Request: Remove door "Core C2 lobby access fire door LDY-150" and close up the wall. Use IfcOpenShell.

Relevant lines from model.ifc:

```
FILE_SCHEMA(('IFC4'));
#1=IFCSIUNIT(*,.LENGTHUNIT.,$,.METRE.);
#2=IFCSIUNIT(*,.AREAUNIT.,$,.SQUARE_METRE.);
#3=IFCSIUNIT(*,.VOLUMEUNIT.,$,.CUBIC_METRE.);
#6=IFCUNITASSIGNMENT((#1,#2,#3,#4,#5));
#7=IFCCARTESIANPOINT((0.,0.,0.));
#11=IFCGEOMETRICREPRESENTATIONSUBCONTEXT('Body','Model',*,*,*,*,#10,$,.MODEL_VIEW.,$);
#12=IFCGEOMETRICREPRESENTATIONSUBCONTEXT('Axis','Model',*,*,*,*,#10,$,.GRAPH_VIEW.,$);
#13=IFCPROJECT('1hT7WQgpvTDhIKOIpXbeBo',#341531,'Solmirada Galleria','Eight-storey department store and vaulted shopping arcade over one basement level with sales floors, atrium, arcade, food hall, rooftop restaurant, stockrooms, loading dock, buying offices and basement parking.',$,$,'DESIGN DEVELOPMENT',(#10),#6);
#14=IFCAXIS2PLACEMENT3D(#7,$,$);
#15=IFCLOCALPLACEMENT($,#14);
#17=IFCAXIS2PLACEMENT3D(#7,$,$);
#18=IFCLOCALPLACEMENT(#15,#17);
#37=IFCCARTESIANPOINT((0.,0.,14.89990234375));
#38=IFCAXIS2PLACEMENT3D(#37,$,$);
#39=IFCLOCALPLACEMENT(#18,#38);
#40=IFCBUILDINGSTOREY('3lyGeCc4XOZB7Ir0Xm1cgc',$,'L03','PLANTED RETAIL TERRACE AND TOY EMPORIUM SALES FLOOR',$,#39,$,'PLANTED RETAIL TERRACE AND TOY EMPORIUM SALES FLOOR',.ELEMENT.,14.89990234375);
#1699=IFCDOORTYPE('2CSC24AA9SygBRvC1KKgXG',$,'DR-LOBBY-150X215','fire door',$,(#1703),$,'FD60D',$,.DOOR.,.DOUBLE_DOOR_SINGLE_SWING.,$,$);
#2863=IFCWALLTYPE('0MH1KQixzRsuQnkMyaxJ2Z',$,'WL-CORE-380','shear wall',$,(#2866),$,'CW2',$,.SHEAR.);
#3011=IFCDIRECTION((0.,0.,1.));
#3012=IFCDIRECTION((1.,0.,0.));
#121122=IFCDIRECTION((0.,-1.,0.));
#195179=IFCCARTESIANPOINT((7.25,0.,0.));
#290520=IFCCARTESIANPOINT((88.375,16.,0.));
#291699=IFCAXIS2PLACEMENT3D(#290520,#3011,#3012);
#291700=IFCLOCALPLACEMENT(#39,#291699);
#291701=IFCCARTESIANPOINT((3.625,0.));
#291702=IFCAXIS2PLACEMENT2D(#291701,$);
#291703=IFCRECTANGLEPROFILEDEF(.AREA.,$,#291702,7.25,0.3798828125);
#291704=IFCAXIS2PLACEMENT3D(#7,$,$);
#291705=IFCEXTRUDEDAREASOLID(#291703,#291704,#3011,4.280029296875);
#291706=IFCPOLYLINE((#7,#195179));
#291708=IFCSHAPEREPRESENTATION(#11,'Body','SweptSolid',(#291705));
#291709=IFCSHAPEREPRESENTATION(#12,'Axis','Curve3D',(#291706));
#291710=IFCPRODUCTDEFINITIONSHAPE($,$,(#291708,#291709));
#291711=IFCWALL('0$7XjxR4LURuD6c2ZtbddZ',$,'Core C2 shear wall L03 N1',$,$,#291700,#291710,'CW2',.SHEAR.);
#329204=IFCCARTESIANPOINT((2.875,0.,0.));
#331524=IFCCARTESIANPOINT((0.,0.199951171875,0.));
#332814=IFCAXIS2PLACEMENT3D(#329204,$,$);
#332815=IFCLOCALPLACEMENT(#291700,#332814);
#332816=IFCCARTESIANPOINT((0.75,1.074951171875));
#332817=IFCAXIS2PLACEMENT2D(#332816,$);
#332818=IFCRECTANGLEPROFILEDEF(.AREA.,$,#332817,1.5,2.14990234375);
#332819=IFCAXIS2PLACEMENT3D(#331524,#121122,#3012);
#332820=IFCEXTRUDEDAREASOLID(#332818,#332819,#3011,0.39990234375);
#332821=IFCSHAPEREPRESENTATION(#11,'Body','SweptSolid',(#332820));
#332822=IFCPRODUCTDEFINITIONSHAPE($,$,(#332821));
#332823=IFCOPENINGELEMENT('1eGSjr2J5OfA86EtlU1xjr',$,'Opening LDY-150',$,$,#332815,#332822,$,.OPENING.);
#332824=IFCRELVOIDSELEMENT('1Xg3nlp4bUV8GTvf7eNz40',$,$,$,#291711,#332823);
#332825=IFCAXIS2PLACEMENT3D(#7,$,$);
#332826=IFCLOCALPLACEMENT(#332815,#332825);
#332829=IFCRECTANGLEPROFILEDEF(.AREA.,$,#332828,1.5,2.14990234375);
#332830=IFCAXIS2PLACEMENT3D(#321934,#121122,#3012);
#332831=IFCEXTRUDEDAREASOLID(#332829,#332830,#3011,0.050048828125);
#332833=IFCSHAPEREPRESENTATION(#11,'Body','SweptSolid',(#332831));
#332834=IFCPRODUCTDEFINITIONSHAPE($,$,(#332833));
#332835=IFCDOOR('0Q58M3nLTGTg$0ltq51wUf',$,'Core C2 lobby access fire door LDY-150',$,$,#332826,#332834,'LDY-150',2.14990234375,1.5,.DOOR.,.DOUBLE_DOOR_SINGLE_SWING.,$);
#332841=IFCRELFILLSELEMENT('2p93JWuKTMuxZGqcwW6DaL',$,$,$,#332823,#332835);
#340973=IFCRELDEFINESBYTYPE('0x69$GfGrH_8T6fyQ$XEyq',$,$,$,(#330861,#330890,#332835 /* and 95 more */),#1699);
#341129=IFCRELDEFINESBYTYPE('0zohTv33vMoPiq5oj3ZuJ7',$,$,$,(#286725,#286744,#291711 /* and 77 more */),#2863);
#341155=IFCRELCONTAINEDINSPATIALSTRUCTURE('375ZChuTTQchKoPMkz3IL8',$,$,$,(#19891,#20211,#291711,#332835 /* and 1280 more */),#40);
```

```python
import ifcopenshell
import ifcopenshell.api.feature
import ifcopenshell.api.root
import ifcopenshell.geom
import ifcopenshell.util.shape

model = ifcopenshell.open("model.ifc")
settings = ifcopenshell.geom.settings()


def volume(element):
    """Net volume in cubic metres, openings subtracted."""
    shape = ifcopenshell.geom.create_shape(settings, element)
    return ifcopenshell.util.shape.get_volume(shape.geometry)


door = model.by_guid("0Q58M3nLTGTg$0ltq51wUf")
opening = door.FillsVoids[0].RelatingOpeningElement
wall = opening.VoidsElements[0].RelatingBuildingElement
before = volume(wall)

ifcopenshell.api.root.remove_product(model, product=door)
ifcopenshell.api.feature.remove_feature(model, feature=opening)

after = volume(wall)

print(f"wall volume {before:.3f} -> {after:.3f} m3")

model.write("model_rev.ifc")
```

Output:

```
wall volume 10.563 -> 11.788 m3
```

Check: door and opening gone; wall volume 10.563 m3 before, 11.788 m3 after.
